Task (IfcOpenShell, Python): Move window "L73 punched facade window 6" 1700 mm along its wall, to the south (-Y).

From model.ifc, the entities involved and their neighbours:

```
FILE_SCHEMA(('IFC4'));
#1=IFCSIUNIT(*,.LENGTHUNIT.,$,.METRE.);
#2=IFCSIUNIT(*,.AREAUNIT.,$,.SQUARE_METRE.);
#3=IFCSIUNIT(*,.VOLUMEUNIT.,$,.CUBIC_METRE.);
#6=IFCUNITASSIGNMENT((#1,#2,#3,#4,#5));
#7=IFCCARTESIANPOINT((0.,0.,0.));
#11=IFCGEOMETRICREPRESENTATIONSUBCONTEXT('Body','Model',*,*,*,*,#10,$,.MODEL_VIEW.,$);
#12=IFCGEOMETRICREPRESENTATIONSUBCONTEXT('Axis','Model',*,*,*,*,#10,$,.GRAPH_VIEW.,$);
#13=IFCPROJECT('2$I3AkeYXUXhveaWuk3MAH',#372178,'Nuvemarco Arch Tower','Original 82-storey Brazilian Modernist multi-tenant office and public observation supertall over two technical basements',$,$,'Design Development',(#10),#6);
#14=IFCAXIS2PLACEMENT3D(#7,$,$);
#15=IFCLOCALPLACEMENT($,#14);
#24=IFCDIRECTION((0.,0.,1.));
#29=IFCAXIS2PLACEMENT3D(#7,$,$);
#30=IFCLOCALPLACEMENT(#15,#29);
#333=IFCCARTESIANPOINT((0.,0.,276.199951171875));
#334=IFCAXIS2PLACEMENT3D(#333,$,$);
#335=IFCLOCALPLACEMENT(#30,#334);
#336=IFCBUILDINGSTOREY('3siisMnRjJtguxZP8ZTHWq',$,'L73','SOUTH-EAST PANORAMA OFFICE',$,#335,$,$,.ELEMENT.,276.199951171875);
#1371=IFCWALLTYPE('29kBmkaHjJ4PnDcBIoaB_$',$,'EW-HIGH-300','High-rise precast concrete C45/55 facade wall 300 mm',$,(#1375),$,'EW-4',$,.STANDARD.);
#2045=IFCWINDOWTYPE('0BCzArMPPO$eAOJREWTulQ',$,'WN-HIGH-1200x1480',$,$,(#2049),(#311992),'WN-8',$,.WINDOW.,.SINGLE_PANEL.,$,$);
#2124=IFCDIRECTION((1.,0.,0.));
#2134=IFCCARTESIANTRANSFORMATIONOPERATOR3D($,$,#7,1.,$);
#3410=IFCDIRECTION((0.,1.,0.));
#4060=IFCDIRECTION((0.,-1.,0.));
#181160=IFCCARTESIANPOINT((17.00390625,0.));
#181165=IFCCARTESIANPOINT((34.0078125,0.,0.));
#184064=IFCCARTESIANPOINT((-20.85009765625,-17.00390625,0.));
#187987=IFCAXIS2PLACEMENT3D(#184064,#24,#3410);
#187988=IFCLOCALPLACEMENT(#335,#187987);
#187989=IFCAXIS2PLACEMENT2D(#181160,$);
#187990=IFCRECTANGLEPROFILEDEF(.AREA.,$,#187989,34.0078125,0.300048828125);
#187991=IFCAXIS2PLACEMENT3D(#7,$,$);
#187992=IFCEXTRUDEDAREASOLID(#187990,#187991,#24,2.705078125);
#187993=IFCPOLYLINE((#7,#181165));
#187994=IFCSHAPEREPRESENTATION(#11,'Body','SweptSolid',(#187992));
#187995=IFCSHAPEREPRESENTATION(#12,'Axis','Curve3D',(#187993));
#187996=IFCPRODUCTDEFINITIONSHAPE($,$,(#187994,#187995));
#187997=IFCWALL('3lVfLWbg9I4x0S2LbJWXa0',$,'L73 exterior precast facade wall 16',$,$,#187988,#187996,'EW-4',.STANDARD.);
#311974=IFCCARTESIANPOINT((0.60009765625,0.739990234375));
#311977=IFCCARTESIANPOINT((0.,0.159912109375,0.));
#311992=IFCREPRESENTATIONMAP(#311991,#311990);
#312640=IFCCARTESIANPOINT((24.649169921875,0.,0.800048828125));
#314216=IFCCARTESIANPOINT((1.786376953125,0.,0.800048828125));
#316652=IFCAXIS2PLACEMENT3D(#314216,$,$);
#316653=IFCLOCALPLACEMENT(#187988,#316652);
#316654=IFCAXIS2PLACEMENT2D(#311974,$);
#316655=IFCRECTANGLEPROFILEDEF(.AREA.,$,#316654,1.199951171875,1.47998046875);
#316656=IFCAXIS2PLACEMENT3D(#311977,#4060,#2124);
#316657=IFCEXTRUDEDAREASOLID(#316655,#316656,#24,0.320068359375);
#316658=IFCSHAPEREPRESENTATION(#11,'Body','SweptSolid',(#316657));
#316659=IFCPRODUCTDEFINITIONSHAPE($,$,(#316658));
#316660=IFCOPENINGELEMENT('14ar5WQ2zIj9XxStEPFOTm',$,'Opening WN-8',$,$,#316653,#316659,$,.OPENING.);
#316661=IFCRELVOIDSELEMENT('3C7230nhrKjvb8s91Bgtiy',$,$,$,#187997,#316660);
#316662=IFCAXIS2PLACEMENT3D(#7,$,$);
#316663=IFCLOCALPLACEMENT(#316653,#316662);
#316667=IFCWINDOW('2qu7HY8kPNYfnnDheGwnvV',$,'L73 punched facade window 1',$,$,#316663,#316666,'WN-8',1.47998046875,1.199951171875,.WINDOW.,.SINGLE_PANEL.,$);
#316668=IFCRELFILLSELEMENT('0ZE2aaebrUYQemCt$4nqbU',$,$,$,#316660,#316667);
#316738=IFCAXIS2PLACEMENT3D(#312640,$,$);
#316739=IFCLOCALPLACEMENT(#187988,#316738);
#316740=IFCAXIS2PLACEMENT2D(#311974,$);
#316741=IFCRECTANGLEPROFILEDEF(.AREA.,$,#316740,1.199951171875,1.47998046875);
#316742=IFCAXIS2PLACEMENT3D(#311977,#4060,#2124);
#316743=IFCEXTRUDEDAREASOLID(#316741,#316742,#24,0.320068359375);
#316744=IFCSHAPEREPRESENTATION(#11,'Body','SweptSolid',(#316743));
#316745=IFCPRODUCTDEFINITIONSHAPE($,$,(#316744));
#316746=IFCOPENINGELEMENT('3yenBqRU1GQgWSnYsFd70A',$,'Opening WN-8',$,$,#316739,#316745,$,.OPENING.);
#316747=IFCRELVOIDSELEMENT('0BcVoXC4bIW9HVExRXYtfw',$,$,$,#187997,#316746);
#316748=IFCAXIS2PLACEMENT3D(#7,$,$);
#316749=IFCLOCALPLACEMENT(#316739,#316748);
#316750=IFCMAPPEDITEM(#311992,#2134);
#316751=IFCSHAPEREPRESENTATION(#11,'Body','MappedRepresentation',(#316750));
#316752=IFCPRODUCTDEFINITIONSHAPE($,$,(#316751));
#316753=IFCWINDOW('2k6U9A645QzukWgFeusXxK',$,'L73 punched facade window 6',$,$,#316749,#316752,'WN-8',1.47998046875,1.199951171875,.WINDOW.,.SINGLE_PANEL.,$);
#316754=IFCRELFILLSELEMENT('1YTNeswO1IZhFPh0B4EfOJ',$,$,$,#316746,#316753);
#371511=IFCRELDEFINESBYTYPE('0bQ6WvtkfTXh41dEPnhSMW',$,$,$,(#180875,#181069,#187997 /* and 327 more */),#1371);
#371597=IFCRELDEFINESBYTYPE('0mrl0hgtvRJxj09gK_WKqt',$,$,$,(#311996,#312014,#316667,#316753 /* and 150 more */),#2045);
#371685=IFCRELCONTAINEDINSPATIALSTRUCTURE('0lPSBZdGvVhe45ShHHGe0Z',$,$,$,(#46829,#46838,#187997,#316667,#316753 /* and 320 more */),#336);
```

```python
import ifcopenshell
import ifcopenshell.api.geometry
import ifcopenshell.util.placement
import ifcopenshell.util.unit

model = ifcopenshell.open("model.ifc")
unit_scale = ifcopenshell.util.unit.calculate_unit_scale(model)

window = model.by_guid("2k6U9A645QzukWgFeusXxK")
opening = window.FillsVoids[0].RelatingOpeningElement
wall = opening.VoidsElements[0].RelatingBuildingElement

wall_matrix = ifcopenshell.util.placement.get_local_placement(wall.ObjectPlacement)
shift = wall_matrix[:3, 0] * -1.7 / unit_scale
before = ifcopenshell.util.placement.get_local_placement(window.ObjectPlacement)[:3, 3].copy()

# The window is placed relative to its opening, so it follows when the opening moves.
matrix = ifcopenshell.util.placement.get_local_placement(opening.ObjectPlacement)
matrix[:3, 3] += shift
ifcopenshell.api.geometry.edit_object_placement(
    model, product=opening, matrix=matrix, is_si=False, should_transform_children=True
)

after = ifcopenshell.util.placement.get_local_placement(window.ObjectPlacement)[:3, 3]
print("window moved by", (after - before).round(3) + 0.0)

model.write("model_updated.ifc")
```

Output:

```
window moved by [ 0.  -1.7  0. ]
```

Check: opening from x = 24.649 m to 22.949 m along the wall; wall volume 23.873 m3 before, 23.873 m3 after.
